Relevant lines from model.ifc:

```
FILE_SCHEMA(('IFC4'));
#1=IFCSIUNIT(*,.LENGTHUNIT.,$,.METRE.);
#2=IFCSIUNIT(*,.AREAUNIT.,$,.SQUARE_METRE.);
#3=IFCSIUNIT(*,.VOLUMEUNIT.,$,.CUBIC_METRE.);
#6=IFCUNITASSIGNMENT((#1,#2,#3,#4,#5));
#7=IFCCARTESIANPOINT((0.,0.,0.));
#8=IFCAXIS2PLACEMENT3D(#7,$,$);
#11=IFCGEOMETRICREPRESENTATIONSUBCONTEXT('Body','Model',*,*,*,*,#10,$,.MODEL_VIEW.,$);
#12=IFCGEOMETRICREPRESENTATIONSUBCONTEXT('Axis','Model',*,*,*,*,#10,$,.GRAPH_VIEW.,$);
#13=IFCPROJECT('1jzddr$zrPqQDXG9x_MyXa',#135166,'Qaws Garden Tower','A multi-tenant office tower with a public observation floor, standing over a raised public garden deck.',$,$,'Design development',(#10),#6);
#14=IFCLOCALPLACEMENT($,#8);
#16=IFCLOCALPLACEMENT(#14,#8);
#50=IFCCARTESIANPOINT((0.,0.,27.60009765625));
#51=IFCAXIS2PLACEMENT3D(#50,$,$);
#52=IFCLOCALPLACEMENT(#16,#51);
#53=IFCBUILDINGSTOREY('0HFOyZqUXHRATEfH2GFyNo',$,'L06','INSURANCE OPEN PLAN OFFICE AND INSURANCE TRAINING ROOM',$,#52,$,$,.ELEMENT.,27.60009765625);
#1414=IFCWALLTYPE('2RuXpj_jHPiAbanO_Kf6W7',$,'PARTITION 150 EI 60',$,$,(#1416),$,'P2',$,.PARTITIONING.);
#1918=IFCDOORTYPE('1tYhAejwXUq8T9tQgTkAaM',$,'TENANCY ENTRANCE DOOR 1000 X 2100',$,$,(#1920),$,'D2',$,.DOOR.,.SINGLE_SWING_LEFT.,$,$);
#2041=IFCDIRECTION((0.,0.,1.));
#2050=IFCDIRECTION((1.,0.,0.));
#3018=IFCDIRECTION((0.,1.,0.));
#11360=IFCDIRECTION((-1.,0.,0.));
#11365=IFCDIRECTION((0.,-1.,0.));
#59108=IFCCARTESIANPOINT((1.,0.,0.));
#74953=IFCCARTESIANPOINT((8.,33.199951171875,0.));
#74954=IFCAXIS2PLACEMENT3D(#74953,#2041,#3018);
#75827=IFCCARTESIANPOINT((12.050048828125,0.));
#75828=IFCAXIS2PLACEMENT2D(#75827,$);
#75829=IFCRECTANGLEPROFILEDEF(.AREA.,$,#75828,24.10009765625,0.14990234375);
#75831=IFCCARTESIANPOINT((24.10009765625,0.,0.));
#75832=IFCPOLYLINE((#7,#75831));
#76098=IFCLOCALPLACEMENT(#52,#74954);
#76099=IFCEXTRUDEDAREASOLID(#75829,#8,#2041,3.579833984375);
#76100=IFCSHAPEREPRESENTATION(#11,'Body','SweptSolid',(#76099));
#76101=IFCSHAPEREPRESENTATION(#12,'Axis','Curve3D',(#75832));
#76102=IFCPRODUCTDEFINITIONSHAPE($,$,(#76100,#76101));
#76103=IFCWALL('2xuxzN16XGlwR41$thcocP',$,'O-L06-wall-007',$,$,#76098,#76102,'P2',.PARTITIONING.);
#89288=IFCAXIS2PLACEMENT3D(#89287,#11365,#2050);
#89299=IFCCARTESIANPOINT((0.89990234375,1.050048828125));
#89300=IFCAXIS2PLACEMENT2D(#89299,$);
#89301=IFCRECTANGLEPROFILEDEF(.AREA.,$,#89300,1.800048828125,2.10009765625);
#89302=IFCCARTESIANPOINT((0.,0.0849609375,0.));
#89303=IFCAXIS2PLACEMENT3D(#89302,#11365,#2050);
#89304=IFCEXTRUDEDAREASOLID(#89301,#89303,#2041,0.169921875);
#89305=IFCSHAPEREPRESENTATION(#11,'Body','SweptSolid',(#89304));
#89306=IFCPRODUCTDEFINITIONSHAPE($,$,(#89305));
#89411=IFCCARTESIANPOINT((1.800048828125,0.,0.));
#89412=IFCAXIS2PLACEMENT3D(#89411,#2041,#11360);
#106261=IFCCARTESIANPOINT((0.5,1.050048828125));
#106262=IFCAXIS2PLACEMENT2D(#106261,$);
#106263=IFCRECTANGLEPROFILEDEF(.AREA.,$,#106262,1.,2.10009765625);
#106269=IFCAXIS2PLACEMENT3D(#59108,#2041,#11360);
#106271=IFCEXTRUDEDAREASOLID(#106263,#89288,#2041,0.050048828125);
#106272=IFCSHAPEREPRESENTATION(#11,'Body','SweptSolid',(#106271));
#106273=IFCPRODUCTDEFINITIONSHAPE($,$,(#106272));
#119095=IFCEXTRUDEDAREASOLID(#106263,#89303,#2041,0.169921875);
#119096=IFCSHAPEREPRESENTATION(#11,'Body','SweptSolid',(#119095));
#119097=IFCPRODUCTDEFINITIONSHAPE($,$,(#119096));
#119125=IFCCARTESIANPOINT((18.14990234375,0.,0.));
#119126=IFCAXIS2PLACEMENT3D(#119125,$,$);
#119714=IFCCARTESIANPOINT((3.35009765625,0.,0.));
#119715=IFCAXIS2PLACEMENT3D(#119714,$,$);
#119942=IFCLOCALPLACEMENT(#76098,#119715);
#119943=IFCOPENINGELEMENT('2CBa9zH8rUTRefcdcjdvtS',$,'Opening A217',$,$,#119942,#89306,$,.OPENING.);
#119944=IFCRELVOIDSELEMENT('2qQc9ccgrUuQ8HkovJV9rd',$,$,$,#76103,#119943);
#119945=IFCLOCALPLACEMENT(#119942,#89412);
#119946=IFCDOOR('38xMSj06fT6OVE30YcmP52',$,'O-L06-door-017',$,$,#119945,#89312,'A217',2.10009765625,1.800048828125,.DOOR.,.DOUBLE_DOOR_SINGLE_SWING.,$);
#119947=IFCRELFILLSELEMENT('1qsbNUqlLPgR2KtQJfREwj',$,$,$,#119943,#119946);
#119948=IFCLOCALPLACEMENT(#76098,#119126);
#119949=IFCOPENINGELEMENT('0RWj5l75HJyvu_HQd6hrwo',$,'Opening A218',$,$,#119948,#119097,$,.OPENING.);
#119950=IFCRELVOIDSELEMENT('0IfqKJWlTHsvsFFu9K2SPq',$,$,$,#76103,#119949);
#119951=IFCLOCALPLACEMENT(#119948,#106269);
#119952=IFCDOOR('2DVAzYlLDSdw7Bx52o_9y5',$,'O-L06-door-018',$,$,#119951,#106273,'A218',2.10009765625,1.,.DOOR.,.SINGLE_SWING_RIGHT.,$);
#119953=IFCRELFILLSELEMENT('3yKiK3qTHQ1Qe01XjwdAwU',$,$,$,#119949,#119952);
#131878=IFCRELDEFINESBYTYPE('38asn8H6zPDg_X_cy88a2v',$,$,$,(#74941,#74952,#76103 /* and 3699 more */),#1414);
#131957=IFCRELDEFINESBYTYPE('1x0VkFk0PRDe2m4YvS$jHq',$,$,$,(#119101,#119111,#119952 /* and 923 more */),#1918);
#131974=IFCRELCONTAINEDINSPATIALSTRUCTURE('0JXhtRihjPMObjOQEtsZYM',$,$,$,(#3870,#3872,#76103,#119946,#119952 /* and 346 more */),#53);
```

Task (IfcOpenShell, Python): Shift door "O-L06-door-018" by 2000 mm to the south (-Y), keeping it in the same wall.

```python
import ifcopenshell
import ifcopenshell.api.geometry
import ifcopenshell.util.placement
import ifcopenshell.util.unit

model = ifcopenshell.open("model.ifc")
unit_scale = ifcopenshell.util.unit.calculate_unit_scale(model)

door = model.by_id(119952)
opening = door.FillsVoids[0].RelatingOpeningElement
wall = opening.VoidsElements[0].RelatingBuildingElement

wall_matrix = ifcopenshell.util.placement.get_local_placement(wall.ObjectPlacement)
shift = wall_matrix[:3, 0] * -2 / unit_scale
before = ifcopenshell.util.placement.get_local_placement(door.ObjectPlacement)[:3, 3].copy()

# The door is placed relative to its opening, so it follows when the opening moves.
matrix = ifcopenshell.util.placement.get_local_placement(opening.ObjectPlacement)
matrix[:3, 3] += shift
ifcopenshell.api.geometry.edit_object_placement(
    model, product=opening, matrix=matrix, is_si=False, should_transform_children=True
)

after = ifcopenshell.util.placement.get_local_placement(door.ObjectPlacement)[:3, 3]
print("door moved by", (after - before).round(3) + 0.0)

model.write("model_rev.ifc")
```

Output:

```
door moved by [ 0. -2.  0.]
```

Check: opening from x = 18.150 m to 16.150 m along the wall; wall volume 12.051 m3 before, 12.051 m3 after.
